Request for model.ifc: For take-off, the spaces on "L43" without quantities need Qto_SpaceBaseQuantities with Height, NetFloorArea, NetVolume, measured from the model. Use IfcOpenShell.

First a look at what the model holds.

```python
import ifcopenshell
import ifcopenshell.util.element
import ifcopenshell.util.unit

model = ifcopenshell.open("model.ifc")
print(model.schema)
for unit_type in ("LENGTHUNIT", "AREAUNIT", "VOLUMEUNIT"):
    print(unit_type, ifcopenshell.util.unit.calculate_unit_scale(model, unit_type))
storey = next(s for s in model.by_type("IfcBuildingStorey") if s.Name == "L43")
spaces = [e for e in ifcopenshell.util.element.get_decomposition(storey) if e.is_a("IfcSpace")]
for e in sorted(spaces, key=lambda e: e.id()):
    print(e.id(), e.is_a(), e.Name, list(ifcopenshell.util.element.get_psets(e, qtos_only=True)), sep=" | ")
```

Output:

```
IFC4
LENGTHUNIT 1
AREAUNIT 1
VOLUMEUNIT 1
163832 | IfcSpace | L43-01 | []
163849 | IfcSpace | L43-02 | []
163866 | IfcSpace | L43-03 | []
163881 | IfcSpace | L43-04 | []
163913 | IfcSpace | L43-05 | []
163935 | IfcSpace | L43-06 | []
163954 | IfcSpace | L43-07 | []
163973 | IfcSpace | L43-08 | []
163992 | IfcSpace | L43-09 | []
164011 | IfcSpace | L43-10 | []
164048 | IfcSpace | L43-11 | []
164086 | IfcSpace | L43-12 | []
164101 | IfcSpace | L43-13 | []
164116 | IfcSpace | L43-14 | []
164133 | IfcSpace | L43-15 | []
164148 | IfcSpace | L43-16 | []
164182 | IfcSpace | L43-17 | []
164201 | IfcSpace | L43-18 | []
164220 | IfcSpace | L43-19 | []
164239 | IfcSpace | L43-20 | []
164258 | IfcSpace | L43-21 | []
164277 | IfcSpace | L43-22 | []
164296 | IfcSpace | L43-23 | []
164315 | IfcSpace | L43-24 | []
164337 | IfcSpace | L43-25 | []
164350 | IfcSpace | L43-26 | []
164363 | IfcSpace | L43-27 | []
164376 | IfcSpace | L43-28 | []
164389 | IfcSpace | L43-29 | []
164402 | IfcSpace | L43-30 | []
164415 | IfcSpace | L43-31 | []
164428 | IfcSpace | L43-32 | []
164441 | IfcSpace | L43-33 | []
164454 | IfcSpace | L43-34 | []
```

```python
import ifcopenshell
import ifcopenshell.api.pset
import ifcopenshell.geom
import ifcopenshell.util.element
import ifcopenshell.util.shape
import ifcopenshell.util.unit

model = ifcopenshell.open("model.ifc")
unit_scale = ifcopenshell.util.unit.calculate_unit_scale(model)
area_scale = ifcopenshell.util.unit.calculate_unit_scale(model, "AREAUNIT")
volume_scale = ifcopenshell.util.unit.calculate_unit_scale(model, "VOLUMEUNIT")
settings = ifcopenshell.geom.settings()

storey = next(s for s in model.by_type("IfcBuildingStorey") if s.Name == "L43")
spaces = [e for e in ifcopenshell.util.element.get_decomposition(storey) if e.is_a("IfcSpace")]

for e in sorted(spaces, key=lambda e: e.id()):
    if ifcopenshell.util.element.get_psets(e, qtos_only=True, should_inherit=False):
        continue
    # Geometry comes back in metres, in the element's own axes.
    shape = ifcopenshell.geom.create_shape(settings, e)
    values = {
        "Height": ifcopenshell.util.shape.get_z(shape.geometry) / unit_scale,
        "NetFloorArea": ifcopenshell.util.shape.get_footprint_area(shape.geometry) / area_scale,
        "NetVolume": ifcopenshell.util.shape.get_volume(shape.geometry) / volume_scale,
    }
    qto = ifcopenshell.api.pset.add_qto(model, product=e, name="Qto_SpaceBaseQuantities")
    ifcopenshell.api.pset.edit_qto(model, qto=qto, properties=values)
    print(e.id(), {k: round(v, 3) for k, v in values.items()})

model.write("model-out.ifc")
```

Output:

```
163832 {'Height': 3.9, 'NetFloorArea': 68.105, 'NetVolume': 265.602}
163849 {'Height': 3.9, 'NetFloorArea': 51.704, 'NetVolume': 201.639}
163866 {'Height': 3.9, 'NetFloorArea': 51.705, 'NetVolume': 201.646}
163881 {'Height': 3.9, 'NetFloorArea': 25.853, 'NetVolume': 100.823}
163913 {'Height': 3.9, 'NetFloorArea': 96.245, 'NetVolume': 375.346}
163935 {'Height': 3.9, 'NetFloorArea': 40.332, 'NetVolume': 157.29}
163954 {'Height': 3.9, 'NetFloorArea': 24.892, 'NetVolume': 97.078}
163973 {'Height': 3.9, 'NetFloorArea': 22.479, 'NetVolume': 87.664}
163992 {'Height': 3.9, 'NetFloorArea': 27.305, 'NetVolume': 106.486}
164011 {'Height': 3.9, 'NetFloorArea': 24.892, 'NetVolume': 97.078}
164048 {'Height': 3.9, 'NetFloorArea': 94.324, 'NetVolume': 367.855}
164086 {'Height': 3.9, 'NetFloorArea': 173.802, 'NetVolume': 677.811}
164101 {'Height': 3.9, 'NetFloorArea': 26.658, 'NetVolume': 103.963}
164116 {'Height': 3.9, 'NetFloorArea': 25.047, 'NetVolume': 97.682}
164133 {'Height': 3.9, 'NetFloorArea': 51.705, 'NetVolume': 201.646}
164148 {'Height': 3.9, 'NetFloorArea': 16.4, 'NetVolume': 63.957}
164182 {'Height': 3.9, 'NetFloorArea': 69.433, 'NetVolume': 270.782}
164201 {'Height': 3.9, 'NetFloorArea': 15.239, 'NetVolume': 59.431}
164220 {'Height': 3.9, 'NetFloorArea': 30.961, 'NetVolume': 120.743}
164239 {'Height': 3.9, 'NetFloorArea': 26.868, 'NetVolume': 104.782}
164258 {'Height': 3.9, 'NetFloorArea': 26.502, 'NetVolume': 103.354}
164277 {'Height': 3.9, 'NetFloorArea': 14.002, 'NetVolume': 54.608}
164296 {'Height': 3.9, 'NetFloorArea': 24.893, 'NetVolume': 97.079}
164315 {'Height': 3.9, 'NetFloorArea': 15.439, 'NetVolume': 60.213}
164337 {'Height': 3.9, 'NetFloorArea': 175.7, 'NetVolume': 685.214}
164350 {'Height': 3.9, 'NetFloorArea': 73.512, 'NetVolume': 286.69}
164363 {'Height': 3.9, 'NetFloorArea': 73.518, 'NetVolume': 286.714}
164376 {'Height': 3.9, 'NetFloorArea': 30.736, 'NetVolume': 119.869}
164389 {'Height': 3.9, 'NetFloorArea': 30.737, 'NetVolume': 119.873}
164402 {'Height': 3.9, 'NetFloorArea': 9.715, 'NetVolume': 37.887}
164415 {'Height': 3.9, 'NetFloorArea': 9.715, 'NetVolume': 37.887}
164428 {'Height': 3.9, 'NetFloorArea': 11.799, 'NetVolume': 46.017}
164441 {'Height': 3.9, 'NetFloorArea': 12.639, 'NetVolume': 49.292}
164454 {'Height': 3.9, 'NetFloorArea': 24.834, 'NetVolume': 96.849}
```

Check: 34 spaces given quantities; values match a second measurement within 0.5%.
